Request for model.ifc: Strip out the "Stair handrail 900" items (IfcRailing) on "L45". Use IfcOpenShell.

First a look at what the model holds.

```python
import ifcopenshell
import ifcopenshell.util.element

model = ifcopenshell.open("model.ifc")
print(model.schema)
storey = next(s for s in model.by_type("IfcBuildingStorey") if s.Name == "L45")
railings = [e for e in ifcopenshell.util.element.get_decomposition(storey) if e.is_a("IfcRailing")]
seen = {}
for e in railings:
    element_type = ifcopenshell.util.element.get_type(e)
    name = element_type.Name if element_type not in (None, e) else None
    seen[name] = seen.get(name, 0) + 1
for name, count in sorted(seen.items(), key=str):
    print(count, "x", name)
```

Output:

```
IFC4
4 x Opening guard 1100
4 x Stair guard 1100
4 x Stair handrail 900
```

```python
import ifcopenshell
import ifcopenshell.api.root
import ifcopenshell.util.element

model = ifcopenshell.open("model.ifc")

storey = next(s for s in model.by_type("IfcBuildingStorey") if s.Name == "L45")
railings = [e for e in ifcopenshell.util.element.get_decomposition(storey) if e.is_a("IfcRailing")]
targets = [e for e in railings if (t := ifcopenshell.util.element.get_type(e)) not in (None, e) and t.Name == "Stair handrail 900"]

for e in targets:
    ifcopenshell.api.root.remove_product(model, product=e)
print(len(targets), "removed")

model.write("model_edited.ifc")
```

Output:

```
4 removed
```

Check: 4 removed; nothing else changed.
